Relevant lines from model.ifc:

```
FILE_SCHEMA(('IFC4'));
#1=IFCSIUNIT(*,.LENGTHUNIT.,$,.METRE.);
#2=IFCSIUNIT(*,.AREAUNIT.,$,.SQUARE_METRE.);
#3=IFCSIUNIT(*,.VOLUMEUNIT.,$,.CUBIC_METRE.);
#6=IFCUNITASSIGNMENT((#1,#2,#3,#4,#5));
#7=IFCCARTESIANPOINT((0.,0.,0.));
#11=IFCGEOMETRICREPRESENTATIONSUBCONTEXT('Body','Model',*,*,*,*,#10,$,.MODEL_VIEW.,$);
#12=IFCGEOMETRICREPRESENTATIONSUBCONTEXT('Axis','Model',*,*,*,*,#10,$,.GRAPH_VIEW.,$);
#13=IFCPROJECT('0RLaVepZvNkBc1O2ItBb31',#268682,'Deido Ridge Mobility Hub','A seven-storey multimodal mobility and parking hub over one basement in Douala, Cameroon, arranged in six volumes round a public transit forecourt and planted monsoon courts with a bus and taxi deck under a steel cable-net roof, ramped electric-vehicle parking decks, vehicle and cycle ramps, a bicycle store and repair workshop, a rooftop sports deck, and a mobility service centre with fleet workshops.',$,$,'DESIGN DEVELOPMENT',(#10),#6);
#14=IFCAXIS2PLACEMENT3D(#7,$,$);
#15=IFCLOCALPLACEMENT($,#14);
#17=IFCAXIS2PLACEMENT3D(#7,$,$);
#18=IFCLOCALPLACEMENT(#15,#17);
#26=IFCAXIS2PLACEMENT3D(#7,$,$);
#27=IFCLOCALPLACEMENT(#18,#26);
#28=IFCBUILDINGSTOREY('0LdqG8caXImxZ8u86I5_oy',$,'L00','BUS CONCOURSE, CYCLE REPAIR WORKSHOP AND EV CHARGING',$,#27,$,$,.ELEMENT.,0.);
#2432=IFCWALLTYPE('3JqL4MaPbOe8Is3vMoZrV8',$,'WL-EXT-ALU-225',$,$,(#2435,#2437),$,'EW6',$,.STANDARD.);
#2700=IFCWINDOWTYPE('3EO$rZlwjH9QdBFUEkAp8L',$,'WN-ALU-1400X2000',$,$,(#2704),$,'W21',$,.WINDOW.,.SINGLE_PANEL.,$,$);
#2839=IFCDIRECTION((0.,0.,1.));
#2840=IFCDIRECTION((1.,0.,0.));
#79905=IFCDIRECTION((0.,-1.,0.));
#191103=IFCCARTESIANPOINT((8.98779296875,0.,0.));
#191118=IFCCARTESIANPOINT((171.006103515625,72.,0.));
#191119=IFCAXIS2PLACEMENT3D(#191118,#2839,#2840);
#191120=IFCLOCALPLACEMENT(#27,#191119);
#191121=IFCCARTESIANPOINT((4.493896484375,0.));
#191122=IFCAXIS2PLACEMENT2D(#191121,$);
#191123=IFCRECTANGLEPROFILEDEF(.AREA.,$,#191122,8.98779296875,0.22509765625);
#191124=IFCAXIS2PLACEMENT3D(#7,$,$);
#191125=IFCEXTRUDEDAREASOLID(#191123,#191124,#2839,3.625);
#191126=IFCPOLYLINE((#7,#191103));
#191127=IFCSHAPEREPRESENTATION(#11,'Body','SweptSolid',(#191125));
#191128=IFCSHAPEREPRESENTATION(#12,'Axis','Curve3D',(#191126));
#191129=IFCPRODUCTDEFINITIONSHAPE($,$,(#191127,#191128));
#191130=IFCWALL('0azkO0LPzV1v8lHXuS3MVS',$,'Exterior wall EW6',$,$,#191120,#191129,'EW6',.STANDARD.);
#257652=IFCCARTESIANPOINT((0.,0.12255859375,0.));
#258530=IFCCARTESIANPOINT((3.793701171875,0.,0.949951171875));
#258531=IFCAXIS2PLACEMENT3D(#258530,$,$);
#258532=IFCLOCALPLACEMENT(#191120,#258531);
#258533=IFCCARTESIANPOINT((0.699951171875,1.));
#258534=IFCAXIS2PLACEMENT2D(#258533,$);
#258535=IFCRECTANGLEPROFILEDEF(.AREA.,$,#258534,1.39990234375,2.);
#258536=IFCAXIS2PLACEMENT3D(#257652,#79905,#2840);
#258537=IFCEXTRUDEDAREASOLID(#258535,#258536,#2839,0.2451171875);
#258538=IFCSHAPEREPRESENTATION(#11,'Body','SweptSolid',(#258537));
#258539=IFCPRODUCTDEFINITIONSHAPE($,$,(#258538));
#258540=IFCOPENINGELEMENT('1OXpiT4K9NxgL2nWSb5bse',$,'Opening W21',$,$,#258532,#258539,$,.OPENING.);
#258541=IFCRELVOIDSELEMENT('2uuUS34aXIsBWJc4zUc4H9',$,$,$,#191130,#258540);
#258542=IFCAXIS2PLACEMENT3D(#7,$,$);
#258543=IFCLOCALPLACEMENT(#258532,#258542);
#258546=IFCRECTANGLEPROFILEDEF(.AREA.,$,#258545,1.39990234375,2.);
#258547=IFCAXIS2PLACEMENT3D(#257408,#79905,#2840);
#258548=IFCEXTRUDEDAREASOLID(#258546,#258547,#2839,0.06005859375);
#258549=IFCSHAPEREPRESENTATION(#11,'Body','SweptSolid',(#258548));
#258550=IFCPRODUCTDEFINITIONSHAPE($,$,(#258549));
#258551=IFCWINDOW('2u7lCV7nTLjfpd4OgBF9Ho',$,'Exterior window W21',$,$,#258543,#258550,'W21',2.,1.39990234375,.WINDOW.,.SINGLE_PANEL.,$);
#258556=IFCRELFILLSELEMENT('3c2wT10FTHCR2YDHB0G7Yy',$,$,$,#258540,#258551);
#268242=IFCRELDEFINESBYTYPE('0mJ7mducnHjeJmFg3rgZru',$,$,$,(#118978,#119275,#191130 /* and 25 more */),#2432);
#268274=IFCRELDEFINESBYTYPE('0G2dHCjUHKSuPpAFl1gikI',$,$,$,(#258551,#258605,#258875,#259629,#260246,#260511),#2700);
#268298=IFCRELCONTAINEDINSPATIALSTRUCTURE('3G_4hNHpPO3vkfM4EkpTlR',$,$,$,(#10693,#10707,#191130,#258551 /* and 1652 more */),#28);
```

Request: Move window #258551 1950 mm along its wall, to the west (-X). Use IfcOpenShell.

```python
import ifcopenshell
import ifcopenshell.api.geometry
import ifcopenshell.util.placement
import ifcopenshell.util.unit

model = ifcopenshell.open("model.ifc")
unit_scale = ifcopenshell.util.unit.calculate_unit_scale(model)

window = model.by_guid("2u7lCV7nTLjfpd4OgBF9Ho")
opening = window.FillsVoids[0].RelatingOpeningElement
wall = opening.VoidsElements[0].RelatingBuildingElement

wall_matrix = ifcopenshell.util.placement.get_local_placement(wall.ObjectPlacement)
shift = wall_matrix[:3, 0] * -1.95 / unit_scale
before = ifcopenshell.util.placement.get_local_placement(window.ObjectPlacement)[:3, 3].copy()

# The window is placed relative to its opening, so it follows when the opening moves.
matrix = ifcopenshell.util.placement.get_local_placement(opening.ObjectPlacement)
matrix[:3, 3] += shift
ifcopenshell.api.geometry.edit_object_placement(
    model, product=opening, matrix=matrix, is_si=False, should_transform_children=True
)

after = ifcopenshell.util.placement.get_local_placement(window.ObjectPlacement)[:3, 3]
print("window moved by", (after - before).round(3) + 0.0)

model.write("model_rev.ifc")
```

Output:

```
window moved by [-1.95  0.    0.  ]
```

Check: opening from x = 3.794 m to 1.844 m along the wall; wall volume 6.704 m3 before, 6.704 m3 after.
